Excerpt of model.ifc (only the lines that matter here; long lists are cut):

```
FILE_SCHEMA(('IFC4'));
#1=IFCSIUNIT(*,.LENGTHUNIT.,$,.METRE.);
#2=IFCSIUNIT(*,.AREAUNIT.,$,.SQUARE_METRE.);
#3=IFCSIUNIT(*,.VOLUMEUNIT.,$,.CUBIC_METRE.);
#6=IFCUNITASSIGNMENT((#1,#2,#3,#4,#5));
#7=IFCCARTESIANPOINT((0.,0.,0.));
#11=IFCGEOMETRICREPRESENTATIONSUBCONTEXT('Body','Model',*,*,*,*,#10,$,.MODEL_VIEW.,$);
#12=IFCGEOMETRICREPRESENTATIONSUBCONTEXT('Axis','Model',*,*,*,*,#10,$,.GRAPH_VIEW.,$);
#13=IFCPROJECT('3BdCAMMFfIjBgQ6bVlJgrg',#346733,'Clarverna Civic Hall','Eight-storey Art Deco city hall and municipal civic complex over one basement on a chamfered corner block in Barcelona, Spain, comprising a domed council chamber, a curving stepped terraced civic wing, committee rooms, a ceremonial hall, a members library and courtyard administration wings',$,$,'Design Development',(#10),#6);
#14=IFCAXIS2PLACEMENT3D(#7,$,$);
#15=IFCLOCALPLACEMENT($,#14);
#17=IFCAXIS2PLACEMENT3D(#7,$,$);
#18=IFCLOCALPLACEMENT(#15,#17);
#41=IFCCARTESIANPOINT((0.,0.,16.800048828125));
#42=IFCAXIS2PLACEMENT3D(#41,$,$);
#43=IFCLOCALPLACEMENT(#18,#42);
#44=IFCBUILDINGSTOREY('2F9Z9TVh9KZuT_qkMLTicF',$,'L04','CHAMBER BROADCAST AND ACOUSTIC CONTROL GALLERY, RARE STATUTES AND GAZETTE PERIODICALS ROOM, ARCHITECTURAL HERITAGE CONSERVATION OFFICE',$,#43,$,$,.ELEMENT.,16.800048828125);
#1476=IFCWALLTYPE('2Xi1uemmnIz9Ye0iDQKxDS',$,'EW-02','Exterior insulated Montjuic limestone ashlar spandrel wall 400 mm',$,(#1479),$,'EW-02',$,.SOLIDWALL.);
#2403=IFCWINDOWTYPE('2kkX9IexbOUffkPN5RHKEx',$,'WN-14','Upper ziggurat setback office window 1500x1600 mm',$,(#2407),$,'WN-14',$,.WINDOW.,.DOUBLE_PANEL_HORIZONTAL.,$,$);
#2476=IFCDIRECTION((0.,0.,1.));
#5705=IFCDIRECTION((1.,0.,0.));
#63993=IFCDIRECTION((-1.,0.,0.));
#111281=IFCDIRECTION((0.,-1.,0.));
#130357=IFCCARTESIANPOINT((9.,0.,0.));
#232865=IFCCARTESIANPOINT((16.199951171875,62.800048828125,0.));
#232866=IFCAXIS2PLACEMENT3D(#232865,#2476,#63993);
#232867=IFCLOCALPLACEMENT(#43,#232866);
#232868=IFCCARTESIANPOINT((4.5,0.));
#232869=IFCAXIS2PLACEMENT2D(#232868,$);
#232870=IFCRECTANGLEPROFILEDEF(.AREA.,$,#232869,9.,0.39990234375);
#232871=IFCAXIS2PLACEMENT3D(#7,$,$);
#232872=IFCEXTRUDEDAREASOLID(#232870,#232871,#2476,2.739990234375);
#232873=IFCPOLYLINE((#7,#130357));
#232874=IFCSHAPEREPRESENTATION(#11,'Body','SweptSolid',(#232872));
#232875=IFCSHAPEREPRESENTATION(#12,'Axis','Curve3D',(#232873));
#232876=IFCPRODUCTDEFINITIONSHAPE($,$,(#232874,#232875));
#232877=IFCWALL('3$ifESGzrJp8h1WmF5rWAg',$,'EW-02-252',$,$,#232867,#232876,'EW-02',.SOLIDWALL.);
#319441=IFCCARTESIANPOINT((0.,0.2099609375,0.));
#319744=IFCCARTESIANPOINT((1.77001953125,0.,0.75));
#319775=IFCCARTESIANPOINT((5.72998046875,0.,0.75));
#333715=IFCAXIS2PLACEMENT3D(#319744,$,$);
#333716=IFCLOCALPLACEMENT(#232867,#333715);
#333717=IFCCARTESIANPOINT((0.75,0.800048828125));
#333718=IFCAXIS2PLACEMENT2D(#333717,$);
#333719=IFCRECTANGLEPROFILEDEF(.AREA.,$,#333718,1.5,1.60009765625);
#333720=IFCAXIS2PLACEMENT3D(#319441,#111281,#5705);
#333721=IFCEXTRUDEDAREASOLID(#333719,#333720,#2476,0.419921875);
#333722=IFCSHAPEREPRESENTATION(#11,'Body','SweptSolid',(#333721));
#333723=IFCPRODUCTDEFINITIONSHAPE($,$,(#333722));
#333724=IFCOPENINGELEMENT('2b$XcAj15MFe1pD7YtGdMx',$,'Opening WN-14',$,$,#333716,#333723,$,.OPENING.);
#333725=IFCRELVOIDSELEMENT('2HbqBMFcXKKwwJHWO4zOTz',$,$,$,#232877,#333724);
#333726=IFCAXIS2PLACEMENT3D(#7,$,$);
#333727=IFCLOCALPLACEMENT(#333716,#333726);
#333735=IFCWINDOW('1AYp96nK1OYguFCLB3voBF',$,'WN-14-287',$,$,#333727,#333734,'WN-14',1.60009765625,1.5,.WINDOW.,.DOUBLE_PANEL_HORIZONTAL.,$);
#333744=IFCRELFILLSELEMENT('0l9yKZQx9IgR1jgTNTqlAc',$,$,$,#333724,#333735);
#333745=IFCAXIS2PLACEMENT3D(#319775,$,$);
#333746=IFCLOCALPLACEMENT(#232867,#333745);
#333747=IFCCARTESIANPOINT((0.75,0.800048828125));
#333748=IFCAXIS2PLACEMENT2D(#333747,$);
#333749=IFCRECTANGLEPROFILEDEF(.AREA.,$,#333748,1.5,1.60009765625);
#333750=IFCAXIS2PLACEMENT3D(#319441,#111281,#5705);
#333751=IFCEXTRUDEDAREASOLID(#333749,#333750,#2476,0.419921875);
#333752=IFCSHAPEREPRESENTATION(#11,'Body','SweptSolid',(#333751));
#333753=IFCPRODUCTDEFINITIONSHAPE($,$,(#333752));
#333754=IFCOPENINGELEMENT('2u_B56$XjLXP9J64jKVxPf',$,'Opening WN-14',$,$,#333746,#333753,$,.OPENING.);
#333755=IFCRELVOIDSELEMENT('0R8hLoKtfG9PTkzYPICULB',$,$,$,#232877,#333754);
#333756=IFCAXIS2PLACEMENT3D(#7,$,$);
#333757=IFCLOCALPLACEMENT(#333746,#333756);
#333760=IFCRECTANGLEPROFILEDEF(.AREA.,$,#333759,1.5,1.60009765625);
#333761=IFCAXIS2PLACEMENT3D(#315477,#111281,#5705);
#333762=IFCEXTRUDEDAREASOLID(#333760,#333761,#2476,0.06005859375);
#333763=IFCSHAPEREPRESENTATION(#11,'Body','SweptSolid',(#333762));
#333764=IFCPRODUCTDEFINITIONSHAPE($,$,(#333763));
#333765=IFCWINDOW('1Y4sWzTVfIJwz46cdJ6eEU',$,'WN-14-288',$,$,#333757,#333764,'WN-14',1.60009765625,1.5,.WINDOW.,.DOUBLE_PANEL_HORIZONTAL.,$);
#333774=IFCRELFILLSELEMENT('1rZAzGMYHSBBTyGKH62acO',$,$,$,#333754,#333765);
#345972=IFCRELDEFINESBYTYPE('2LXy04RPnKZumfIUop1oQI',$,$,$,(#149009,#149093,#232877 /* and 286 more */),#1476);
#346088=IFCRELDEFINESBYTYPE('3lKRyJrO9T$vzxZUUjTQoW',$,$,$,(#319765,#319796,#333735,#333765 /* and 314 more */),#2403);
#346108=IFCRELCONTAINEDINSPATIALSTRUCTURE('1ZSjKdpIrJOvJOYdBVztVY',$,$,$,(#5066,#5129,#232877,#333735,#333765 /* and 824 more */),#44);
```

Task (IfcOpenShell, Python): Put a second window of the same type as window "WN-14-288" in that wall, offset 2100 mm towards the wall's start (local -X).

```python
import ifcopenshell
import ifcopenshell.api.feature
import ifcopenshell.api.geometry
import ifcopenshell.api.root
import ifcopenshell.geom
import ifcopenshell.util.element
import ifcopenshell.util.placement
import ifcopenshell.util.shape
import ifcopenshell.util.unit

model = ifcopenshell.open("model.ifc")
unit_scale = ifcopenshell.util.unit.calculate_unit_scale(model)
settings = ifcopenshell.geom.settings()


def volume(element):
    """Net volume in cubic metres, openings subtracted."""
    shape = ifcopenshell.geom.create_shape(settings, element)
    return ifcopenshell.util.shape.get_volume(shape.geometry)


window = model.by_guid("1Y4sWzTVfIJwz46cdJ6eEU")
opening = window.FillsVoids[0].RelatingOpeningElement
wall = opening.VoidsElements[0].RelatingBuildingElement
before = volume(wall)
shift = ifcopenshell.util.placement.get_local_placement(wall.ObjectPlacement)[:3, 0] * -2.1 / unit_scale

# copy_class copies the void relationship, type, container and properties, but no geometry.
new_opening = ifcopenshell.api.root.copy_class(model, product=opening)
new_opening.Representation = ifcopenshell.util.element.copy_deep(
    model, opening.Representation, exclude=["IfcGeometricRepresentationContext", "IfcRepresentationMap"]
)
new_window = ifcopenshell.api.root.copy_class(model, product=window)
new_window.Representation = ifcopenshell.util.element.copy_deep(
    model, window.Representation, exclude=["IfcGeometricRepresentationContext", "IfcRepresentationMap"]
)
new_window.Tag = None
ifcopenshell.api.feature.add_filling(model, opening=new_opening, element=new_window)

for old, new in ((opening, new_opening), (window, new_window)):
    matrix = ifcopenshell.util.placement.get_local_placement(old.ObjectPlacement)
    matrix[:3, 3] += shift
    ifcopenshell.api.geometry.edit_object_placement(model, product=new, matrix=matrix, is_si=False)

after = volume(wall)

print(f"wall volume {before:.3f} -> {after:.3f} m3")

model.write("model_edited.ifc")
```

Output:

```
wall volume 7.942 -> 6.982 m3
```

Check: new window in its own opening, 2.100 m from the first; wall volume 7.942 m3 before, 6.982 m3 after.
